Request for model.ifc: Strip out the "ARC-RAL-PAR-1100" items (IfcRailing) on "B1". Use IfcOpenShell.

First a look at what the model holds.

```python
import ifcopenshell
import ifcopenshell.util.element

model = ifcopenshell.open("model.ifc")
print(model.schema)
storey = next(s for s in model.by_type("IfcBuildingStorey") if s.Name == "B1")
railings = [e for e in ifcopenshell.util.element.get_decomposition(storey) if e.is_a("IfcRailing")]
seen = {}
for e in railings:
    element_type = ifcopenshell.util.element.get_type(e)
    name = element_type.Name if element_type not in (None, e) else None
    seen[name] = seen.get(name, 0) + 1
for name, count in sorted(seen.items(), key=str):
    print(count, "x", name)
```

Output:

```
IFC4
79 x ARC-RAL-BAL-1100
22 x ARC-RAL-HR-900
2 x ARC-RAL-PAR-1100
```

```python
import ifcopenshell
import ifcopenshell.api.root
import ifcopenshell.util.element

model = ifcopenshell.open("model.ifc")

storey = next(s for s in model.by_type("IfcBuildingStorey") if s.Name == "B1")
railings = [e for e in ifcopenshell.util.element.get_decomposition(storey) if e.is_a("IfcRailing")]
targets = [e for e in railings if (t := ifcopenshell.util.element.get_type(e)) not in (None, e) and t.Name == "ARC-RAL-PAR-1100"]

for e in targets:
    ifcopenshell.api.root.remove_product(model, product=e)
print(len(targets), "removed")

model.write("model-out.ifc")
```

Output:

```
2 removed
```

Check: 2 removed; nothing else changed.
